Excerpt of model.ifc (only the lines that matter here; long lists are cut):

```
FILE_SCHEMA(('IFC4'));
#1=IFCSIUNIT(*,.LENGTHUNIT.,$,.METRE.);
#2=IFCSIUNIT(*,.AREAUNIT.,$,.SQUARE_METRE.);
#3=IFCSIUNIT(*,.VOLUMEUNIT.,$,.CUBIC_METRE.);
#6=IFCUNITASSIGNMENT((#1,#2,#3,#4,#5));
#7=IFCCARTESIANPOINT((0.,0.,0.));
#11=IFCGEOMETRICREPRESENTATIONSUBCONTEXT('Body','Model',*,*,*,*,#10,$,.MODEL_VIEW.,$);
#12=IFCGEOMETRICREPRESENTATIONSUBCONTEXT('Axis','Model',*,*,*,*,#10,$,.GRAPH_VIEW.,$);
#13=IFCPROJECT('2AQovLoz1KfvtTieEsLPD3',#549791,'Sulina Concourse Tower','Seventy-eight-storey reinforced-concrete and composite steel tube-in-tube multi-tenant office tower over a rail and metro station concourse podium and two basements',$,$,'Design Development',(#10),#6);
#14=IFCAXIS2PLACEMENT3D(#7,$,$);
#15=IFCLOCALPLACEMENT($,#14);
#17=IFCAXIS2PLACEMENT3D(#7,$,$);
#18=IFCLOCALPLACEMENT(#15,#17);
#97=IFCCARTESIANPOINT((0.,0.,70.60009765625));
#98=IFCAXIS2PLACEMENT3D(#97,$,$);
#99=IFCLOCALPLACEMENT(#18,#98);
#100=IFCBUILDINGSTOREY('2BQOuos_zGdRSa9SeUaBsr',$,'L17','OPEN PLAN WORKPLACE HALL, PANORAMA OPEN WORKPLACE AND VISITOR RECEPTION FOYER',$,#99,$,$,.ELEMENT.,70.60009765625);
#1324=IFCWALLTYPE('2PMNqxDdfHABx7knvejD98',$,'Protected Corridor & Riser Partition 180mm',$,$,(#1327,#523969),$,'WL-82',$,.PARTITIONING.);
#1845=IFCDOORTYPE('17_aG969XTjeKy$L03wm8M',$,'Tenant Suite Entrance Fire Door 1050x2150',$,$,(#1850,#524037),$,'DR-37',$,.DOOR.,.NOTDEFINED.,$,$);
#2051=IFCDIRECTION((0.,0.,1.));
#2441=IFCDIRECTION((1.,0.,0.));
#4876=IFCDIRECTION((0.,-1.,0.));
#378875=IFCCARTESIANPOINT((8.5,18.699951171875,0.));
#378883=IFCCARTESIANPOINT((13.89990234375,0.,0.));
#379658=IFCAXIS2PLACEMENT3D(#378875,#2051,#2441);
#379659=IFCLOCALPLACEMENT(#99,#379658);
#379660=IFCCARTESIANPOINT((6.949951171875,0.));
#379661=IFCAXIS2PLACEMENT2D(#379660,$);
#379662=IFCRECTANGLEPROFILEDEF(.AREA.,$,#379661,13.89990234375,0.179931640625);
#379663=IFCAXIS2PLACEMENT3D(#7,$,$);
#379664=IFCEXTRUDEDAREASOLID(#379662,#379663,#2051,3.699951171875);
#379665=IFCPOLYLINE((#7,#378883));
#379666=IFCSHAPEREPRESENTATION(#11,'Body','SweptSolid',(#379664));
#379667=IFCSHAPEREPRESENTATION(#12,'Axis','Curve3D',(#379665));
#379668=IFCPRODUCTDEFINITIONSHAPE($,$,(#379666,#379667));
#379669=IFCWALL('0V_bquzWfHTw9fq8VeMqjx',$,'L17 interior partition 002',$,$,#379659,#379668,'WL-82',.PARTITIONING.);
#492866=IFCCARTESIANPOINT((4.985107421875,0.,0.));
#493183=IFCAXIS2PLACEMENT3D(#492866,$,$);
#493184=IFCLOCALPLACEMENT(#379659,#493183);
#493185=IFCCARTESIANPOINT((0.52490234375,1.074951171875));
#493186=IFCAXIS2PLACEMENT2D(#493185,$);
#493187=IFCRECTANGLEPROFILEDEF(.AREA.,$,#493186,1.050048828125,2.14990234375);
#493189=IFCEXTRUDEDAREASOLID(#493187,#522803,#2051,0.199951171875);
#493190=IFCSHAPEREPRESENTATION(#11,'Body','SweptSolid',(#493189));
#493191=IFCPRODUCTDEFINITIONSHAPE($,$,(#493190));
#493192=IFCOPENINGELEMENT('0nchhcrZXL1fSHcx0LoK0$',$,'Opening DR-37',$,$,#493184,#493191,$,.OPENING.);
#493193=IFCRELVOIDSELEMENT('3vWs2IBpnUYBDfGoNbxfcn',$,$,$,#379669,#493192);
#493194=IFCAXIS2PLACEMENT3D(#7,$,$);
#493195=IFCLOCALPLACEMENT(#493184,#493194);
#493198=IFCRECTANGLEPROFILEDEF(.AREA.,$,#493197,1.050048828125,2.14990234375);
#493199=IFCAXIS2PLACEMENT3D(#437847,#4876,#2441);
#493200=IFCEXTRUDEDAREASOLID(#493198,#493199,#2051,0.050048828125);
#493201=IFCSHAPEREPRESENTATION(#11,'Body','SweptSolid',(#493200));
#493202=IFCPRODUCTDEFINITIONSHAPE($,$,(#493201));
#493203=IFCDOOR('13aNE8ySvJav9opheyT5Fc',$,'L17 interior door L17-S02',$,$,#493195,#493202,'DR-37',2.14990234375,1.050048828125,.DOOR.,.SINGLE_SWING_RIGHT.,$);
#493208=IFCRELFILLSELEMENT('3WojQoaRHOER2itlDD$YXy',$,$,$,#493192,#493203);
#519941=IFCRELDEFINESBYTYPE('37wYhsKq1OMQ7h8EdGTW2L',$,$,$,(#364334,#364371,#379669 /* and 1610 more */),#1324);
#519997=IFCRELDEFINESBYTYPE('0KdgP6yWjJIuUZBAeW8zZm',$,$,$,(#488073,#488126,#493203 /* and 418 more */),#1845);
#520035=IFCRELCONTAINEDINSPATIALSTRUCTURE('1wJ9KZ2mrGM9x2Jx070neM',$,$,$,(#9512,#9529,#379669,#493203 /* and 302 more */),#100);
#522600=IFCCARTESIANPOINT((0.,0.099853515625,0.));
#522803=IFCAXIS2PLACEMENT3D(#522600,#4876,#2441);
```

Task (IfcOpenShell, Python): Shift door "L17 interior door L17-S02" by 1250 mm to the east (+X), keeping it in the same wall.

```python
import ifcopenshell
import ifcopenshell.api.geometry
import ifcopenshell.util.placement
import ifcopenshell.util.unit

model = ifcopenshell.open("model.ifc")
unit_scale = ifcopenshell.util.unit.calculate_unit_scale(model)

door = model.by_id(493203)
opening = door.FillsVoids[0].RelatingOpeningElement
wall = opening.VoidsElements[0].RelatingBuildingElement

wall_matrix = ifcopenshell.util.placement.get_local_placement(wall.ObjectPlacement)
shift = wall_matrix[:3, 0] * 1.25 / unit_scale
before = ifcopenshell.util.placement.get_local_placement(door.ObjectPlacement)[:3, 3].copy()

# The door is placed relative to its opening, so it follows when the opening moves.
matrix = ifcopenshell.util.placement.get_local_placement(opening.ObjectPlacement)
matrix[:3, 3] += shift
ifcopenshell.api.geometry.edit_object_placement(
    model, product=opening, matrix=matrix, is_si=False, should_transform_children=True
)

after = ifcopenshell.util.placement.get_local_placement(door.ObjectPlacement)[:3, 3]
print("door moved by", (after - before).round(3) + 0.0)

model.write("model_updated.ifc")
```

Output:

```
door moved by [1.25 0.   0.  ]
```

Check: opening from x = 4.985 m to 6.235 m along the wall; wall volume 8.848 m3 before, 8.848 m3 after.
